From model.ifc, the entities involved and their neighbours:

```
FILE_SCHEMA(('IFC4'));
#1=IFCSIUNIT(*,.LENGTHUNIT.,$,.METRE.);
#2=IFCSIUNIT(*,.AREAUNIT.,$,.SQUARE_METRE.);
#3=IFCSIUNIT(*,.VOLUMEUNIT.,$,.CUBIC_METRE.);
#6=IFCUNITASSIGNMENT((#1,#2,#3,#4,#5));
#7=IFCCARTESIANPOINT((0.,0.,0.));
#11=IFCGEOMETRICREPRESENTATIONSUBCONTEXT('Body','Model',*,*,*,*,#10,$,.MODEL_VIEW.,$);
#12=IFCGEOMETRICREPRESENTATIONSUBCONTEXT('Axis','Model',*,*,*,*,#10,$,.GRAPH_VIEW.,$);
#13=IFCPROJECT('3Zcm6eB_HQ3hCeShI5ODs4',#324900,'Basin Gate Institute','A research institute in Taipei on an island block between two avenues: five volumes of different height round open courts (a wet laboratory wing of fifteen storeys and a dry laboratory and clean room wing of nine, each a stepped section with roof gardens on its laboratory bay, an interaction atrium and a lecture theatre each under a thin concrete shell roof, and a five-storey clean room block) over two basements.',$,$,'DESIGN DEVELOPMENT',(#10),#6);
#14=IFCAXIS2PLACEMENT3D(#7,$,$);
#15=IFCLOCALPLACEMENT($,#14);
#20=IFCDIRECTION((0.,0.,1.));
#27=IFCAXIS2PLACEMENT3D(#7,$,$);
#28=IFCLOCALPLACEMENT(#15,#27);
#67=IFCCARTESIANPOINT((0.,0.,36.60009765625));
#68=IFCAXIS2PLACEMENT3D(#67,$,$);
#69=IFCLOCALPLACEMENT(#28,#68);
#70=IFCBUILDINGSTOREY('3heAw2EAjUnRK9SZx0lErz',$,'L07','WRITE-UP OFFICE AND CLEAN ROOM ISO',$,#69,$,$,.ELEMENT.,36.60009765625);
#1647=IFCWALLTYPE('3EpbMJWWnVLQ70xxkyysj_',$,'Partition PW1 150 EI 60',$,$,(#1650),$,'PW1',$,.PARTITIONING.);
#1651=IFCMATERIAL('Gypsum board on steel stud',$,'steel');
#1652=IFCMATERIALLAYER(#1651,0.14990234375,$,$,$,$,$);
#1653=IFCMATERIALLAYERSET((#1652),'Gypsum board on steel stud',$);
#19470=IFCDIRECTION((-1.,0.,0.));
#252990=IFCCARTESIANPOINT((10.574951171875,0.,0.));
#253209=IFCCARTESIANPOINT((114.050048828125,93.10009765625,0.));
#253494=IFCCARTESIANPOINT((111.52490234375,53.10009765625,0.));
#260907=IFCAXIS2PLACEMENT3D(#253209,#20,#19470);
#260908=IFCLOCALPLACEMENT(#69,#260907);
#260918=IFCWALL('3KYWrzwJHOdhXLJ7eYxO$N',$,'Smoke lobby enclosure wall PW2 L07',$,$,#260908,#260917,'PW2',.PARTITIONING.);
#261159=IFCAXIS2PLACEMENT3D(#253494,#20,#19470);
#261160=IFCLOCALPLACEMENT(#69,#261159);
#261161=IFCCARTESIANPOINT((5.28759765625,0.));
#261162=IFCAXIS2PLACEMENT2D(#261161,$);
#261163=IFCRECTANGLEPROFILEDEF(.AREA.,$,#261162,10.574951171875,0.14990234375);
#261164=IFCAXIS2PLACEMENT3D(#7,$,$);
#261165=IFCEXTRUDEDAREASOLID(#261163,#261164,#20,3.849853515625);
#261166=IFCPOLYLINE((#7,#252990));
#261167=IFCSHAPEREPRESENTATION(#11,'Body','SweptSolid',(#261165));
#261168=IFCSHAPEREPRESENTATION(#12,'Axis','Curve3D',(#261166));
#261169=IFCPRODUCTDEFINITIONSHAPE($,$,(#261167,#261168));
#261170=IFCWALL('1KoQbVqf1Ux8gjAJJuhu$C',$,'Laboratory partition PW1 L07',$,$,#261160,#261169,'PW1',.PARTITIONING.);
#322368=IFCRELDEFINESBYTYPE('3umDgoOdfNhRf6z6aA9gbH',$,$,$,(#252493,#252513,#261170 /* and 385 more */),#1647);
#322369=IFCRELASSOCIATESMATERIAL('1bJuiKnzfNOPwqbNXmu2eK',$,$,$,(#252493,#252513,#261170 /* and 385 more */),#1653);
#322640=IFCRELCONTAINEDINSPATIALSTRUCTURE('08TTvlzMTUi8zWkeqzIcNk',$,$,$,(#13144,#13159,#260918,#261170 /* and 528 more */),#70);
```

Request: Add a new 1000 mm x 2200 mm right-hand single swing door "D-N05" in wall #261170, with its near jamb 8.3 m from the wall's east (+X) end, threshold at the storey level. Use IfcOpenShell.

```python
import numpy as np
import ifcopenshell
import ifcopenshell.api.feature
import ifcopenshell.api.geometry
import ifcopenshell.api.root
import ifcopenshell.api.spatial
import ifcopenshell.geom
import ifcopenshell.util.element
import ifcopenshell.util.placement
import ifcopenshell.util.representation
import ifcopenshell.util.shape
import ifcopenshell.util.unit

model = ifcopenshell.open("model.ifc")
unit_scale = ifcopenshell.util.unit.calculate_unit_scale(model)
settings = ifcopenshell.geom.settings()


def volume(element):
    """Net volume in cubic metres, openings subtracted."""
    shape = ifcopenshell.geom.create_shape(settings, element)
    return ifcopenshell.util.shape.get_volume(shape.geometry)


wall = model.by_guid("1KoQbVqf1Ux8gjAJJuhu$C")
storey = ifcopenshell.util.element.get_container(wall, ifc_class="IfcBuildingStorey")
context = ifcopenshell.util.representation.get_context(model, "Model", "Body", "MODEL_VIEW")
before = volume(wall)

width, height, from_end, sill = 1, 2.2, 8.3, 0.0  # metres

# The wall runs along its own X axis, and the end named is its -X end.
wall_shape = ifcopenshell.geom.create_shape(settings, wall)
x, y, z = ifcopenshell.util.shape.get_vertices(wall_shape.geometry).T
start = x.min() + from_end
face, thickness = float(y.min()), float(y.max() - y.min())
wall_matrix = ifcopenshell.util.placement.get_local_placement(wall.ObjectPlacement)
level = ifcopenshell.util.placement.get_local_placement(storey.ObjectPlacement)[2, 3]


def in_wall(x, y):
    """Placement at x, y metres in the wall's axes, at sill height."""
    matrix = wall_matrix.copy()
    matrix[:, 3] = wall_matrix @ np.array([x / unit_scale, y / unit_scale, 0.0, 1.0])
    matrix[2, 3] = level + sill / unit_scale
    return matrix


# Opening: a box that overshoots both wall faces by 50 mm.
opening = ifcopenshell.api.root.create_entity(model, ifc_class="IfcOpeningElement", predefined_type="OPENING")
box = ifcopenshell.api.geometry.add_wall_representation(
    model, context=context, length=width, height=height, thickness=thickness + 0.1
)
ifcopenshell.api.geometry.assign_representation(model, product=opening, representation=box)
ifcopenshell.api.geometry.edit_object_placement(model, product=opening, matrix=in_wall(start, face - 0.05), is_si=False)
ifcopenshell.api.feature.add_feature(model, feature=opening, element=wall)

door = ifcopenshell.api.root.create_entity(model, ifc_class="IfcDoor", name="D-N05", predefined_type="DOOR")
door.OverallWidth, door.OverallHeight = width / unit_scale, height / unit_scale
door.OperationType = "SINGLE_SWING_RIGHT"
body = ifcopenshell.api.geometry.add_door_representation(
    model,
    context=context,
    overall_width=door.OverallWidth,
    overall_height=door.OverallHeight,
    operation_type="SINGLE_SWING_RIGHT",
    lining_properties={"LiningDepth": thickness / unit_scale, "ThresholdDepth": thickness / unit_scale},
)
ifcopenshell.api.geometry.assign_representation(model, product=door, representation=body)
ifcopenshell.api.spatial.assign_container(model, products=[door], relating_structure=storey)
ifcopenshell.api.feature.add_filling(model, opening=opening, element=door)

# The lining spans the wall, so the door starts at the wall face.
ifcopenshell.api.geometry.edit_object_placement(model, product=door, matrix=in_wall(start, face), is_si=False)

after = volume(wall)

print(f"wall volume {before:.3f} -> {after:.3f} m3")

model.write("model-out.ifc")
```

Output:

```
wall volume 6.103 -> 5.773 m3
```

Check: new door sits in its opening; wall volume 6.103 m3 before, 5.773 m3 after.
